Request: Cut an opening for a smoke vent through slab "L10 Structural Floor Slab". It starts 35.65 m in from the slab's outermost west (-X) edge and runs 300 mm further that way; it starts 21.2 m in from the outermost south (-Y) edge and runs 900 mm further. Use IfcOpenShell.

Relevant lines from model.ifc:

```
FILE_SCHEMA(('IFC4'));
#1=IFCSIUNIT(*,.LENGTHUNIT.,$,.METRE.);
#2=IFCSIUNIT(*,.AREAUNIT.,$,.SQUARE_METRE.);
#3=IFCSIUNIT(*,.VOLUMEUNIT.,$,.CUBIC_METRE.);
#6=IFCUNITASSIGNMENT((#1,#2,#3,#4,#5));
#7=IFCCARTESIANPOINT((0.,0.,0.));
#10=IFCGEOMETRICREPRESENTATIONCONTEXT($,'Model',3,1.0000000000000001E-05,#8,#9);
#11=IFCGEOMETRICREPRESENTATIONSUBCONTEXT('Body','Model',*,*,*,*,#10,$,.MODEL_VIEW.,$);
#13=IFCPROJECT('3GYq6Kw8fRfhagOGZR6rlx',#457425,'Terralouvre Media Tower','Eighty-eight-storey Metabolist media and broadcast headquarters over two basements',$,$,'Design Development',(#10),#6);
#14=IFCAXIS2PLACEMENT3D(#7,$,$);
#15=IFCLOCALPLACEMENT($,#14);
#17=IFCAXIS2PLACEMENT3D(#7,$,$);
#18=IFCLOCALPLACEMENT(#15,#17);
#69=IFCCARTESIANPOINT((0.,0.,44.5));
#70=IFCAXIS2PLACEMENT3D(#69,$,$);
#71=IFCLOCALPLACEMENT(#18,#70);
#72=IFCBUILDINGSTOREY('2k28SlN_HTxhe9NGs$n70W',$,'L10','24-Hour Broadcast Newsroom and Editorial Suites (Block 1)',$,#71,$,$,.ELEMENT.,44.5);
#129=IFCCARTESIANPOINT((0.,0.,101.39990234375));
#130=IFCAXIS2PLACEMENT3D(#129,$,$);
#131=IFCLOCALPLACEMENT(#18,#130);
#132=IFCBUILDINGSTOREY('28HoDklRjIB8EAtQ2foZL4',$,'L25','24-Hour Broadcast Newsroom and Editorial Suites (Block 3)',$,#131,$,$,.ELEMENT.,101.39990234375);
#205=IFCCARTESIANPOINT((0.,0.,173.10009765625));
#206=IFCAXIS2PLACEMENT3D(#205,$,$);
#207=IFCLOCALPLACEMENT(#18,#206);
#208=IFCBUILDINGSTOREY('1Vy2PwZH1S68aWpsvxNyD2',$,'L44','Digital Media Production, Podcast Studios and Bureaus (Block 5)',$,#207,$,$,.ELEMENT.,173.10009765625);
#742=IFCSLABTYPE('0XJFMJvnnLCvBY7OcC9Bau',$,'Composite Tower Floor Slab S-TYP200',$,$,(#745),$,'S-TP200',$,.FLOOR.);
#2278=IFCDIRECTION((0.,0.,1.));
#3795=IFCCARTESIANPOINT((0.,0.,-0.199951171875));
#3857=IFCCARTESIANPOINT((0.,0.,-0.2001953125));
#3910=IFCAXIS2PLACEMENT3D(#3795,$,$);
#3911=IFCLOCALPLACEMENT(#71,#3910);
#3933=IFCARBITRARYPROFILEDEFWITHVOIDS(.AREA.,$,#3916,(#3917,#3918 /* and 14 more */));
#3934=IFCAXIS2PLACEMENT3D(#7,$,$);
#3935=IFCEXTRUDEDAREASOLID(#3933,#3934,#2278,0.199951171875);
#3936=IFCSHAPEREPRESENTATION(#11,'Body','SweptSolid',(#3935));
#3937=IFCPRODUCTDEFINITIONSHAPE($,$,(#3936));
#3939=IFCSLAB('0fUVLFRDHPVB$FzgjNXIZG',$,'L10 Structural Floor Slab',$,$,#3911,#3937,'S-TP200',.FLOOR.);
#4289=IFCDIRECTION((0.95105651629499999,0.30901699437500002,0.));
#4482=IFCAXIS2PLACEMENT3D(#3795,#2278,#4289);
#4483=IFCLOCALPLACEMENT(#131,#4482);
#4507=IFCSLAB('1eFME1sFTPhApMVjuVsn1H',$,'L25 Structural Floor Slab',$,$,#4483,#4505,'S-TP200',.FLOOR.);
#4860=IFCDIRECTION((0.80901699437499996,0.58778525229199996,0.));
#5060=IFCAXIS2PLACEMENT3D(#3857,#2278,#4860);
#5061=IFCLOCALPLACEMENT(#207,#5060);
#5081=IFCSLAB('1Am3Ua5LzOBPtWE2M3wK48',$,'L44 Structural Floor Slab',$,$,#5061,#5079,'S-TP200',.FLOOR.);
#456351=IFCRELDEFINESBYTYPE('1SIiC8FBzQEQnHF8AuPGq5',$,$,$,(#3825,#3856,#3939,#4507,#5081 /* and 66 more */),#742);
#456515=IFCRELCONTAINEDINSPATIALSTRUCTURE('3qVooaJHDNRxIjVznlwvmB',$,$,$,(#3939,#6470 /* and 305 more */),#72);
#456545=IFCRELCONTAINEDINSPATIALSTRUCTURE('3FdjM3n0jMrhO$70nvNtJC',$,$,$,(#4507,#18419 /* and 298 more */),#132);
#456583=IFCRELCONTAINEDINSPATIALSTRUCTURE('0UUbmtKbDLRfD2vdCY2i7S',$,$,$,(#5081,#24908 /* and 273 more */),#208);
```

```python
import numpy as np
import ifcopenshell
import ifcopenshell.api.feature
import ifcopenshell.api.geometry
import ifcopenshell.api.root
import ifcopenshell.geom
import ifcopenshell.util.placement
import ifcopenshell.util.representation
import ifcopenshell.util.shape
import ifcopenshell.util.unit

model = ifcopenshell.open("model.ifc")
unit_scale = ifcopenshell.util.unit.calculate_unit_scale(model)
settings = ifcopenshell.geom.settings()


def volume(element):
    """Net volume in cubic metres, openings subtracted."""
    shape = ifcopenshell.geom.create_shape(settings, element)
    return ifcopenshell.util.shape.get_volume(shape.geometry)


slab = model.by_guid("0fUVLFRDHPVB$FzgjNXIZG")
before = volume(slab)

# Extent in the slab's own axes, in metres. The edges named are its -X and -Y sides.
slab_shape = ifcopenshell.geom.create_shape(settings, slab)
vertices = ifcopenshell.util.shape.get_vertices(slab_shape.geometry)
x_min, y_min, bottom = vertices.min(axis=0)
top = vertices[:, 2].max()

opening = ifcopenshell.api.root.create_entity(model, ifc_class="IfcOpeningElement", name="Smoke vent opening", predefined_type="OPENING")
context = ifcopenshell.util.representation.get_context(model, "Model", "Body", "MODEL_VIEW")
width, depth = 0.3, 0.9
outline = [(0.0, 0.0), (width, 0.0), (width, depth), (0.0, depth), (0.0, 0.0)]
# Overshoot both faces by 50 mm so the cut is clean.
shape = ifcopenshell.api.geometry.add_slab_representation(
    model, context=context, depth=top - bottom + 0.1, polyline=outline
)
ifcopenshell.api.geometry.assign_representation(model, product=opening, representation=shape)

matrix = ifcopenshell.util.placement.get_local_placement(slab.ObjectPlacement)
matrix[:, 3] = matrix @ np.append(np.array([x_min + 35.65, y_min + 21.2, bottom - 0.05]) / unit_scale, 1.0)
ifcopenshell.api.geometry.edit_object_placement(model, product=opening, matrix=matrix, is_si=False)
ifcopenshell.api.feature.add_feature(model, feature=opening, element=slab)

after = volume(slab)

print(f"slab volume {before:.3f} -> {after:.3f} m3")

model.write("model_rev.ifc")
```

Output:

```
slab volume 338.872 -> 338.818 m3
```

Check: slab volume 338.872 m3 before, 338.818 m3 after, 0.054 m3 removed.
